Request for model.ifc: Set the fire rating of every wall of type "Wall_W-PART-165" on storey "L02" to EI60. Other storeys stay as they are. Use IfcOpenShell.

First a look at what the model holds.

```python
import ifcopenshell
import ifcopenshell.util.element

model = ifcopenshell.open("model.ifc")
print(model.schema)
storey = next(s for s in model.by_type("IfcBuildingStorey") if s.Name == "L02")
walls = [e for e in ifcopenshell.util.element.get_decomposition(storey) if e.is_a("IfcWall")]
seen = {}
for e in walls:
    element_type = ifcopenshell.util.element.get_type(e)
    key = (element_type.Name if element_type != e and element_type else None, ifcopenshell.util.element.get_pset(e, "Pset_WallCommon", "FireRating"))
    seen[key] = seen.get(key, 0) + 1
for (name, value), count in sorted(seen.items(), key=str):
    print(count, "x", name, "|", value)
```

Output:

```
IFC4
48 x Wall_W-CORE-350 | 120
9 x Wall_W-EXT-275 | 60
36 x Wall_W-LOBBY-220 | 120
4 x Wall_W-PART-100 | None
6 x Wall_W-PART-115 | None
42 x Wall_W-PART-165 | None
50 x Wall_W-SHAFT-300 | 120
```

```python
import ifcopenshell
import ifcopenshell.api.pset
import ifcopenshell.util.element

model = ifcopenshell.open("model.ifc")

storey = next(s for s in model.by_type("IfcBuildingStorey") if s.Name == "L02")
walls = [e for e in ifcopenshell.util.element.get_decomposition(storey) if e.is_a("IfcWall")]

count = 0
for e in walls:
    element_type = ifcopenshell.util.element.get_type(e)
    if element_type in (None, e) or element_type.Name != "Wall_W-PART-165":
        continue
    # add_pset returns the element's existing set when there is one.
    pset = ifcopenshell.api.pset.add_pset(model, product=e, name="Pset_WallCommon")
    ifcopenshell.api.pset.edit_pset(model, pset=pset, properties={"FireRating": "EI60"})
    count += 1

print(count, "walls updated")

model.write("model_v2.ifc")
```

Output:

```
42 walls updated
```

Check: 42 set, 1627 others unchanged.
